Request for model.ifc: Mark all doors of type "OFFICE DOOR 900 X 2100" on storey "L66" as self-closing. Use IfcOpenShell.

First a look at what the model holds.

```python
import ifcopenshell
import ifcopenshell.util.element

model = ifcopenshell.open("model.ifc")
print(model.schema)
storey = next(s for s in model.by_type("IfcBuildingStorey") if s.Name == "L66")
doors = [e for e in ifcopenshell.util.element.get_decomposition(storey) if e.is_a("IfcDoor")]
seen = {}
for e in doors:
    element_type = ifcopenshell.util.element.get_type(e)
    key = (element_type.Name if element_type != e and element_type else None, ifcopenshell.util.element.get_pset(e, "Pset_DoorCommon", "SelfClosing"))
    seen[key] = seen.get(key, 0) + 1
for (name, value), count in sorted(seen.items(), key=str):
    print(count, "x", name, "|", value)
```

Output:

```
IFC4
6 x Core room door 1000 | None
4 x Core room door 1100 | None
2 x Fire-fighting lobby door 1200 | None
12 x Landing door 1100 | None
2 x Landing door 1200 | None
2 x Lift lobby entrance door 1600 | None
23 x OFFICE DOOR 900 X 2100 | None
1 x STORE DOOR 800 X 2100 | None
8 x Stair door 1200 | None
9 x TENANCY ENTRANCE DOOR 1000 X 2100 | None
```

```python
import ifcopenshell
import ifcopenshell.api.pset
import ifcopenshell.util.element

model = ifcopenshell.open("model.ifc")

storey = next(s for s in model.by_type("IfcBuildingStorey") if s.Name == "L66")
doors = [e for e in ifcopenshell.util.element.get_decomposition(storey) if e.is_a("IfcDoor")]

count = 0
for e in doors:
    element_type = ifcopenshell.util.element.get_type(e)
    if element_type in (None, e) or element_type.Name != "OFFICE DOOR 900 X 2100":
        continue
    found = ifcopenshell.util.element.get_pset(e, "Pset_DoorCommon", should_inherit=False)
    if found:
        pset = model.by_id(found["id"])
        if len(ifcopenshell.util.element.get_elements_by_pset(pset)) > 1:
            pset = ifcopenshell.api.pset.unshare_pset(model, products=[e], pset=pset)[0]
    else:
        pset = ifcopenshell.api.pset.add_pset(model, product=e, name="Pset_DoorCommon")
    ifcopenshell.api.pset.edit_pset(model, pset=pset, properties={"SelfClosing": True})
    count += 1

print(count, "doors updated")

model.write("model-out.ifc")
```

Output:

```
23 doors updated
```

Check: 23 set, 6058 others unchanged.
